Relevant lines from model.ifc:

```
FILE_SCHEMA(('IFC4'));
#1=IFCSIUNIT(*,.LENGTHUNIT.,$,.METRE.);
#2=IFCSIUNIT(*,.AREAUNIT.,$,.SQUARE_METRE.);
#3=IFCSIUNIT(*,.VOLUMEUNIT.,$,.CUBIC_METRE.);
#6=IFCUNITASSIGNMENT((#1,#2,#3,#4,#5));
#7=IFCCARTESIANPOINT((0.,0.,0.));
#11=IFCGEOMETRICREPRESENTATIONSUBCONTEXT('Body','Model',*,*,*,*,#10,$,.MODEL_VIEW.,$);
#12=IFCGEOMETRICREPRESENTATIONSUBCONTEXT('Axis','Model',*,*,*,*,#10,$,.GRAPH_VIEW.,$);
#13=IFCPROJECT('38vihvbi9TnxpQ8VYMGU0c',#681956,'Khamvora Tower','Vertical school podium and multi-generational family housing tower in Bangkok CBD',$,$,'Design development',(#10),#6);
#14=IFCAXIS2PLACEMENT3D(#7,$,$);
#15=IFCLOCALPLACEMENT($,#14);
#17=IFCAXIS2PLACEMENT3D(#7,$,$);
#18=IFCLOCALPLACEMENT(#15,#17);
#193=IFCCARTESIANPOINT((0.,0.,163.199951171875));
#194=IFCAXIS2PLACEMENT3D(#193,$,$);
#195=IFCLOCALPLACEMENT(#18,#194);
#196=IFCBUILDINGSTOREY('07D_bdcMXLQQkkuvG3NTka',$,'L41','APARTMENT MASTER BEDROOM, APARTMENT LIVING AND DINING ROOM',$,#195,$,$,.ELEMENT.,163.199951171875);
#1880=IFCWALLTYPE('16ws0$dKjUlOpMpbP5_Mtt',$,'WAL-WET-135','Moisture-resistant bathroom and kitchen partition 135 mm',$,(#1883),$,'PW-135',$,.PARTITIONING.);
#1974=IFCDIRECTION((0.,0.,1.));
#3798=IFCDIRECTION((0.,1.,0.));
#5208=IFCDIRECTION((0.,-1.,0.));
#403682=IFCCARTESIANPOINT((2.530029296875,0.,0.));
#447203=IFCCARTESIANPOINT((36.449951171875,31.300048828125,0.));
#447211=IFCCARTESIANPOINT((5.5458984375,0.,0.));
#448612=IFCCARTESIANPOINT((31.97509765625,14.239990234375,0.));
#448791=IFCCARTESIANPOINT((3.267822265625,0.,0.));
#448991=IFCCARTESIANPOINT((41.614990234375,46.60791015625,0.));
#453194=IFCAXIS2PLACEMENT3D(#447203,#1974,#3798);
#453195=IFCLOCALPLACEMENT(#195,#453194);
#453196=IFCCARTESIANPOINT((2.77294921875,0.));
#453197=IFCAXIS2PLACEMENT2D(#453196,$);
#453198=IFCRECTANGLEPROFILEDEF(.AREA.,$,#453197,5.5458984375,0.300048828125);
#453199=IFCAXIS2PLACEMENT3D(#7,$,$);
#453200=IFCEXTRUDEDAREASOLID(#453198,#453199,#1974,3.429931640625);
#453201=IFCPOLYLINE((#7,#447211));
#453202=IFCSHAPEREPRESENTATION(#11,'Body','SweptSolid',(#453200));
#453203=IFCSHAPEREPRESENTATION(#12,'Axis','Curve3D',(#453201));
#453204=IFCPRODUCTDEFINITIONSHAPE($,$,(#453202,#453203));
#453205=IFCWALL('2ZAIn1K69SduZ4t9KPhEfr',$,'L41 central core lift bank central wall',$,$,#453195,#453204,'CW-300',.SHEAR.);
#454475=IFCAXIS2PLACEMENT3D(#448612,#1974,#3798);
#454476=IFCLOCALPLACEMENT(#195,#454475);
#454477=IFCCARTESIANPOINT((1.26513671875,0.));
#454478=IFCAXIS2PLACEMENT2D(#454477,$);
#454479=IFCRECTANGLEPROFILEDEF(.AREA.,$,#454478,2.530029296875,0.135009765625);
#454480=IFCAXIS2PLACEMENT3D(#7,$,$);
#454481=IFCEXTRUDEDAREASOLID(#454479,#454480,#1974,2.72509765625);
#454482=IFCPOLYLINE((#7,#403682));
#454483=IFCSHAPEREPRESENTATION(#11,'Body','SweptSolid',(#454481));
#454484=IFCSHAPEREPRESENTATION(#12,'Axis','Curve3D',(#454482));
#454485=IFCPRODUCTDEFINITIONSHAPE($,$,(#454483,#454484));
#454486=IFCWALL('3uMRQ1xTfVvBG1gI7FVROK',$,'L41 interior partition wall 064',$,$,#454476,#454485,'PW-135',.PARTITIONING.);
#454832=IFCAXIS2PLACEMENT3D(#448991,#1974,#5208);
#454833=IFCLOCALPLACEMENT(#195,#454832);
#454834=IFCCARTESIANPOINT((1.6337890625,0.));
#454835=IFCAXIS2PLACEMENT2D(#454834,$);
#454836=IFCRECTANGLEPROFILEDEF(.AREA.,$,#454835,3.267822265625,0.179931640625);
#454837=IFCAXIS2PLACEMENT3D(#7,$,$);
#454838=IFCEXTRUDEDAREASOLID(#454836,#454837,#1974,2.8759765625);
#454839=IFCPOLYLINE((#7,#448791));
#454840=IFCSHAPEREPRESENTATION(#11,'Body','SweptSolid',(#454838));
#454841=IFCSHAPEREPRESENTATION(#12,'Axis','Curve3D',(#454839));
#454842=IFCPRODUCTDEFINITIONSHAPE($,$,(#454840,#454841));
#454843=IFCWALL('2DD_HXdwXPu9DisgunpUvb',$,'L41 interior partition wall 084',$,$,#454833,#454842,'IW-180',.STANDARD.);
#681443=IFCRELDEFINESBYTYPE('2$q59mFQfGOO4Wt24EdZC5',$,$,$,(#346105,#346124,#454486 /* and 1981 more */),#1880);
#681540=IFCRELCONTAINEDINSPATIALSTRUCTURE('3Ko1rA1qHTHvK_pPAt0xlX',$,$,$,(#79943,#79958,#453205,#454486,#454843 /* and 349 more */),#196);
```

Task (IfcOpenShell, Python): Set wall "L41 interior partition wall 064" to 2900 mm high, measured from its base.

```python
import ifcopenshell
import ifcopenshell.geom
import ifcopenshell.util.representation
import ifcopenshell.util.shape
import ifcopenshell.util.unit

model = ifcopenshell.open("model.ifc")
unit_scale = ifcopenshell.util.unit.calculate_unit_scale(model)
settings = ifcopenshell.geom.settings()


def volume(element):
    """Net volume in cubic metres, openings subtracted."""
    shape = ifcopenshell.geom.create_shape(settings, element)
    return ifcopenshell.util.shape.get_volume(shape.geometry)


wall = model.by_id(454486)
before = volume(wall)

body = ifcopenshell.util.representation.get_representation(wall, "Model", "Body")
solid = body.Items[0]
old_height = solid.Depth
solid.Depth = 2.9 / unit_scale
after = volume(wall)

print(f"height {old_height:g} -> {solid.Depth:g}, volume {before:.3f} -> {after:.3f} m3")

model.write("model_rev.ifc")
```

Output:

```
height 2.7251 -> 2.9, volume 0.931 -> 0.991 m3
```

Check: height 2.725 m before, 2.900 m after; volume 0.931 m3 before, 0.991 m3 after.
